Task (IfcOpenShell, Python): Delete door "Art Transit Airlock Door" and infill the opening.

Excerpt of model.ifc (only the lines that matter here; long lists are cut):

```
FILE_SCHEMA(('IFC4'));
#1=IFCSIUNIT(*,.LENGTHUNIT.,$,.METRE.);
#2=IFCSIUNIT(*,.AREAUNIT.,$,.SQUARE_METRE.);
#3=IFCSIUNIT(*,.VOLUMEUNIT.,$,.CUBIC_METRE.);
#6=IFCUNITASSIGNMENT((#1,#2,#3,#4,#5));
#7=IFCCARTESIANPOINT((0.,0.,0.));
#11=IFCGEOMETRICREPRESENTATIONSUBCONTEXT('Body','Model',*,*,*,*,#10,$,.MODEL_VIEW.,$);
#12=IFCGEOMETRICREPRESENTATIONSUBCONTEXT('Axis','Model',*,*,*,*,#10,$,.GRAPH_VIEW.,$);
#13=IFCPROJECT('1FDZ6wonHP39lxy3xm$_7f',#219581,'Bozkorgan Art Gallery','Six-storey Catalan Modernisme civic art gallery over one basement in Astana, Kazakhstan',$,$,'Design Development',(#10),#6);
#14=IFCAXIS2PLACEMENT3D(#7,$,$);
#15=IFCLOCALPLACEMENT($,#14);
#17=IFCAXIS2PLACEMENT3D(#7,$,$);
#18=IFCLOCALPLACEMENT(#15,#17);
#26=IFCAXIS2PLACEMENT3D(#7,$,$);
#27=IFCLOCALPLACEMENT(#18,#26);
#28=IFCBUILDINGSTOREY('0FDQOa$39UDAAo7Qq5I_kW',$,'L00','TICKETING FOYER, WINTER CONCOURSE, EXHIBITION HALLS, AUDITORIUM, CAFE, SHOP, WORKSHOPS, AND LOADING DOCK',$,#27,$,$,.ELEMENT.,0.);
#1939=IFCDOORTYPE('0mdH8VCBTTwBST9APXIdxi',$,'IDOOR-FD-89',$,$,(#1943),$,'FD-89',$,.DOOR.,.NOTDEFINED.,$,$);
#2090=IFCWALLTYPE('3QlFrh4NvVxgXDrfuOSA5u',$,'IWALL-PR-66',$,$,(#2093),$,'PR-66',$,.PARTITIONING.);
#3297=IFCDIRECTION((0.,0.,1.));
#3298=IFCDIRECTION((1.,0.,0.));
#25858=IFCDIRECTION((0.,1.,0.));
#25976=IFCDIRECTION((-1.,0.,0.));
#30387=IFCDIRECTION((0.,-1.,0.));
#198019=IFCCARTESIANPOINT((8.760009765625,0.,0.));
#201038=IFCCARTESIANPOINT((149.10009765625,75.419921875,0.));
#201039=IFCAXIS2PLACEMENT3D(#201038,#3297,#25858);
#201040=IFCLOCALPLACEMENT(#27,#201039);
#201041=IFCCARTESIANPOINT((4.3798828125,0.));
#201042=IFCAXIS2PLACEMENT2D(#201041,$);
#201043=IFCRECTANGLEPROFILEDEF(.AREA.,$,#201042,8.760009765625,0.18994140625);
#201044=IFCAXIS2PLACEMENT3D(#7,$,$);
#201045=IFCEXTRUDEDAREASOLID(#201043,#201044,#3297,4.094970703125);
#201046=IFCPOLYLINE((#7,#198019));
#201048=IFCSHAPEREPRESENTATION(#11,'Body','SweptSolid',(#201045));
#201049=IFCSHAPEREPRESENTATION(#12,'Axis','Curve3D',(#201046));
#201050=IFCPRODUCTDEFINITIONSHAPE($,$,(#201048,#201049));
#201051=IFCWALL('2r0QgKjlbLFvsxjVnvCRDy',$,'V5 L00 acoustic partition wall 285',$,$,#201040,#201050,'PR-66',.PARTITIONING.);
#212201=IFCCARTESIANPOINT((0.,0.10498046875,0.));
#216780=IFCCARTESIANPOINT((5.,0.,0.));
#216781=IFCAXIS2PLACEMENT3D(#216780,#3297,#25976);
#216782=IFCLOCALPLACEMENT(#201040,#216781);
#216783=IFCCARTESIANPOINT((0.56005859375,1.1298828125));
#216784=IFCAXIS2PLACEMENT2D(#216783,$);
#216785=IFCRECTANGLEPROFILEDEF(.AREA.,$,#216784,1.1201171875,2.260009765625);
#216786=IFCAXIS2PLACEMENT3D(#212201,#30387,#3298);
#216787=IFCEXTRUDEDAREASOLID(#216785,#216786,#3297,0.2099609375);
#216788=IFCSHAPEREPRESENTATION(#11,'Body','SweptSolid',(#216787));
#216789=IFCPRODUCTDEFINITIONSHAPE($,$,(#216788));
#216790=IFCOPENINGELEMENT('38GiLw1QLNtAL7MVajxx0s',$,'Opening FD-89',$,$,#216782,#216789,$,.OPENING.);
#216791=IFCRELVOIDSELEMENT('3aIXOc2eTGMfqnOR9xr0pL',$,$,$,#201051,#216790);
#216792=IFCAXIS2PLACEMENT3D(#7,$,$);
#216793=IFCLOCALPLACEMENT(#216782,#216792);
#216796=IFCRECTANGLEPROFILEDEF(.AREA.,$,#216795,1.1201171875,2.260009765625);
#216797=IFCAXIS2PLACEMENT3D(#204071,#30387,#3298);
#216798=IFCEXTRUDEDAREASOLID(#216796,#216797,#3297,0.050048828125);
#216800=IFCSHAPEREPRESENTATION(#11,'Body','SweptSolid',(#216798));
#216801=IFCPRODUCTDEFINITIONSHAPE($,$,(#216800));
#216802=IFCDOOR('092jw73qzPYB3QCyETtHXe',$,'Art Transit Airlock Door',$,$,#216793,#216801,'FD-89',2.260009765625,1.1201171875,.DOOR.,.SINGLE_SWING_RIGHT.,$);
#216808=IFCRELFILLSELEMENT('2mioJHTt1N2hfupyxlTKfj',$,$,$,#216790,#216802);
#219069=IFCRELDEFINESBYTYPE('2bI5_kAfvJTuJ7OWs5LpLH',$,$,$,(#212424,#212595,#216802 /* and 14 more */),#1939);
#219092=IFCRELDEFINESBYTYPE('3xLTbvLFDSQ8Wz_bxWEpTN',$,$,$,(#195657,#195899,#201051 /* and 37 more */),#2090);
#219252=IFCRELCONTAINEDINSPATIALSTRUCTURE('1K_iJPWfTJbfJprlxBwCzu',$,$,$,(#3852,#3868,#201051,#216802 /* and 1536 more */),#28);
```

```python
import ifcopenshell
import ifcopenshell.api.feature
import ifcopenshell.api.root
import ifcopenshell.geom
import ifcopenshell.util.shape

model = ifcopenshell.open("model.ifc")
settings = ifcopenshell.geom.settings()


def volume(element):
    """Net volume in cubic metres, openings subtracted."""
    shape = ifcopenshell.geom.create_shape(settings, element)
    return ifcopenshell.util.shape.get_volume(shape.geometry)


door = model.by_id(216802)
opening = door.FillsVoids[0].RelatingOpeningElement
wall = opening.VoidsElements[0].RelatingBuildingElement
before = volume(wall)

ifcopenshell.api.root.remove_product(model, product=door)
ifcopenshell.api.feature.remove_feature(model, feature=opening)

after = volume(wall)

print(f"wall volume {before:.3f} -> {after:.3f} m3")

model.write("model_updated.ifc")
```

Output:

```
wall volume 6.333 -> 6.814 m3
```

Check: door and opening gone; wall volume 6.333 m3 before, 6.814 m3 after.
